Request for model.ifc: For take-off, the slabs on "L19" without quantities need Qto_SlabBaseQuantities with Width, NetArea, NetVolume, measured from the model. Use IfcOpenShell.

First a look at what the model holds.

```python
import ifcopenshell
import ifcopenshell.util.element
import ifcopenshell.util.unit

model = ifcopenshell.open("model.ifc")
print(model.schema)
for unit_type in ("LENGTHUNIT", "AREAUNIT", "VOLUMEUNIT"):
    print(unit_type, ifcopenshell.util.unit.calculate_unit_scale(model, unit_type))
storey = next(s for s in model.by_type("IfcBuildingStorey") if s.Name == "L19")
slabs = [e for e in ifcopenshell.util.element.get_decomposition(storey) if e.is_a("IfcSlab")]
for e in sorted(slabs, key=lambda e: e.id()):
    print(e.id(), e.is_a(), e.Name, list(ifcopenshell.util.element.get_psets(e, qtos_only=True)), sep=" | ")
```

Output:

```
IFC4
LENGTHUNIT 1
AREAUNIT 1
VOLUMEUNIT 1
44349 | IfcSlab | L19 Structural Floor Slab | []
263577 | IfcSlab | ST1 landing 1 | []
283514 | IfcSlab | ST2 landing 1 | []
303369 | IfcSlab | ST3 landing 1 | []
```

```python
import ifcopenshell
import ifcopenshell.api.pset
import ifcopenshell.geom
import ifcopenshell.util.element
import ifcopenshell.util.shape
import ifcopenshell.util.unit

model = ifcopenshell.open("model.ifc")
unit_scale = ifcopenshell.util.unit.calculate_unit_scale(model)
area_scale = ifcopenshell.util.unit.calculate_unit_scale(model, "AREAUNIT")
volume_scale = ifcopenshell.util.unit.calculate_unit_scale(model, "VOLUMEUNIT")
settings = ifcopenshell.geom.settings()

storey = next(s for s in model.by_type("IfcBuildingStorey") if s.Name == "L19")
slabs = [e for e in ifcopenshell.util.element.get_decomposition(storey) if e.is_a("IfcSlab")]

for e in sorted(slabs, key=lambda e: e.id()):
    if ifcopenshell.util.element.get_psets(e, qtos_only=True, should_inherit=False):
        continue
    # Geometry comes back in metres, in the element's own axes.
    shape = ifcopenshell.geom.create_shape(settings, e)
    values = {
        "Width": ifcopenshell.util.shape.get_z(shape.geometry) / unit_scale,
        "NetArea": ifcopenshell.util.shape.get_footprint_area(shape.geometry) / area_scale,
        "NetVolume": ifcopenshell.util.shape.get_volume(shape.geometry) / volume_scale,
    }
    qto = ifcopenshell.api.pset.add_qto(model, product=e, name="Qto_SlabBaseQuantities")
    ifcopenshell.api.pset.edit_qto(model, qto=qto, properties=values)
    print(e.id(), {k: round(v, 3) for k, v in values.items()})

model.write("model_rev.ifc")
```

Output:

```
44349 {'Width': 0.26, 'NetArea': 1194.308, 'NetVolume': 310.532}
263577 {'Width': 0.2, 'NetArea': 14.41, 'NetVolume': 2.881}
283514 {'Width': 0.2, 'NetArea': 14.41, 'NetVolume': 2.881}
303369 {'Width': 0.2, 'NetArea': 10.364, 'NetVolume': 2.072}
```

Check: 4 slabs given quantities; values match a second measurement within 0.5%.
